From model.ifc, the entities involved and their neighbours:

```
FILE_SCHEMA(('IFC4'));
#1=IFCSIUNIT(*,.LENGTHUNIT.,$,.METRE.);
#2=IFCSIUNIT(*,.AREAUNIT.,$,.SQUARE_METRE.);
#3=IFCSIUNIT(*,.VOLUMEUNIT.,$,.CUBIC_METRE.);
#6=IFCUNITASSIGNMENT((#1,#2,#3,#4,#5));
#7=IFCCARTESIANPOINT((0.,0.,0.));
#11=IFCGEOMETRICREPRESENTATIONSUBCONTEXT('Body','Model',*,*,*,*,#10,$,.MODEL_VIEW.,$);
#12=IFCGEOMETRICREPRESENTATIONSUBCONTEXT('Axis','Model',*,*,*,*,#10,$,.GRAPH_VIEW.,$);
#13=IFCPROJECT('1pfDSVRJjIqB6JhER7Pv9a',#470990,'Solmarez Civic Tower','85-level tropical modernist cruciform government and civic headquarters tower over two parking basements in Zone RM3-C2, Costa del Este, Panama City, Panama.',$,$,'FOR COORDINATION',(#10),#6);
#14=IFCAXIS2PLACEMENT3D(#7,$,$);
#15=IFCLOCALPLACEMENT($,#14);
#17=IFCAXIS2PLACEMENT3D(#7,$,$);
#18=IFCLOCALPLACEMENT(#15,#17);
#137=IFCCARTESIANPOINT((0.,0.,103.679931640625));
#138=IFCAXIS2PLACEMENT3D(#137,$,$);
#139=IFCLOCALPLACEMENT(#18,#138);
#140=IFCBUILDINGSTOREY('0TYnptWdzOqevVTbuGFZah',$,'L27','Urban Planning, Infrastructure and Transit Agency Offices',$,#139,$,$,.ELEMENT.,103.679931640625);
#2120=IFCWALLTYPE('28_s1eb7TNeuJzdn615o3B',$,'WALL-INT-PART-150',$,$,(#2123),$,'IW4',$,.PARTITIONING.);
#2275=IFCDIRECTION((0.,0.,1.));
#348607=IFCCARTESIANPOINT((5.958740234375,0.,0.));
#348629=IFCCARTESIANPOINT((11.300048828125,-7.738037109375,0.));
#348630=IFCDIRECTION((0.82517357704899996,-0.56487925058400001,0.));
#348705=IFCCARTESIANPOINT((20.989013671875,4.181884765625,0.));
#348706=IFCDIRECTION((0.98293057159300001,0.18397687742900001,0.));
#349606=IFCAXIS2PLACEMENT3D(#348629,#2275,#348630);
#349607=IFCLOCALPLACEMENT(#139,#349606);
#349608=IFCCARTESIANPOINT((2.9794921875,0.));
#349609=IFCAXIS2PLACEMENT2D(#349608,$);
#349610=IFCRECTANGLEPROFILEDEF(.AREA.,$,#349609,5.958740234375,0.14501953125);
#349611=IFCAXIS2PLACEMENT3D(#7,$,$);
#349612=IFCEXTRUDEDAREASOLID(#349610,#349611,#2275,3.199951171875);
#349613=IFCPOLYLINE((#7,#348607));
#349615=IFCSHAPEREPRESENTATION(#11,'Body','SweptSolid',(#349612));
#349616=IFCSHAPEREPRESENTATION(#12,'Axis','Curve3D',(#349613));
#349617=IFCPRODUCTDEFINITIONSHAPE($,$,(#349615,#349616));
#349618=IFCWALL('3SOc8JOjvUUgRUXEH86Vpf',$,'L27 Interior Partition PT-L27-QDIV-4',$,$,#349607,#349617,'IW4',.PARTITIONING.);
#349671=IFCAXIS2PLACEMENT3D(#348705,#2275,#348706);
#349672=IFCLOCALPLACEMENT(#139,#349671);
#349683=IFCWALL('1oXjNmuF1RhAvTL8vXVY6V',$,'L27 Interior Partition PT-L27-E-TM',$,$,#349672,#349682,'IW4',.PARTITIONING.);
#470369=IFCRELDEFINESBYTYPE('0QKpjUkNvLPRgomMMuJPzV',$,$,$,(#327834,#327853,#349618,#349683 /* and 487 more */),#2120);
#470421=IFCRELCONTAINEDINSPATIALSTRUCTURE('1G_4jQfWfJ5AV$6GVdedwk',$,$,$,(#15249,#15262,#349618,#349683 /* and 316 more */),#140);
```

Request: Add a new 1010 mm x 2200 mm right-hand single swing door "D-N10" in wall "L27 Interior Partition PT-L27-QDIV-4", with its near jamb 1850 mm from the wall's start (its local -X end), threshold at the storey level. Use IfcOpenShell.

```python
import numpy as np
import ifcopenshell
import ifcopenshell.api.feature
import ifcopenshell.api.geometry
import ifcopenshell.api.root
import ifcopenshell.api.spatial
import ifcopenshell.geom
import ifcopenshell.util.element
import ifcopenshell.util.placement
import ifcopenshell.util.representation
import ifcopenshell.util.shape
import ifcopenshell.util.unit

model = ifcopenshell.open("model.ifc")
unit_scale = ifcopenshell.util.unit.calculate_unit_scale(model)
settings = ifcopenshell.geom.settings()


def volume(element):
    """Net volume in cubic metres, openings subtracted."""
    shape = ifcopenshell.geom.create_shape(settings, element)
    return ifcopenshell.util.shape.get_volume(shape.geometry)


wall = model.by_id(349618)
storey = ifcopenshell.util.element.get_container(wall, ifc_class="IfcBuildingStorey")
context = ifcopenshell.util.representation.get_context(model, "Model", "Body", "MODEL_VIEW")
before = volume(wall)

width, height, from_end, sill = 1.01, 2.2, 1.85, 0.0  # metres

# The wall runs along its own X axis, and the end named is its -X end.
wall_shape = ifcopenshell.geom.create_shape(settings, wall)
x, y, z = ifcopenshell.util.shape.get_vertices(wall_shape.geometry).T
start = x.min() + from_end
face, thickness = float(y.min()), float(y.max() - y.min())
wall_matrix = ifcopenshell.util.placement.get_local_placement(wall.ObjectPlacement)
level = ifcopenshell.util.placement.get_local_placement(storey.ObjectPlacement)[2, 3]


def in_wall(x, y):
    """Placement at x, y metres in the wall's axes, at sill height."""
    matrix = wall_matrix.copy()
    matrix[:, 3] = wall_matrix @ np.array([x / unit_scale, y / unit_scale, 0.0, 1.0])
    matrix[2, 3] = level + sill / unit_scale
    return matrix


# Opening: a box that overshoots both wall faces by 50 mm.
opening = ifcopenshell.api.root.create_entity(model, ifc_class="IfcOpeningElement", predefined_type="OPENING")
box = ifcopenshell.api.geometry.add_wall_representation(
    model, context=context, length=width, height=height, thickness=thickness + 0.1
)
ifcopenshell.api.geometry.assign_representation(model, product=opening, representation=box)
ifcopenshell.api.geometry.edit_object_placement(model, product=opening, matrix=in_wall(start, face - 0.05), is_si=False)
ifcopenshell.api.feature.add_feature(model, feature=opening, element=wall)

door = ifcopenshell.api.root.create_entity(model, ifc_class="IfcDoor", name="D-N10", predefined_type="DOOR")
door.OverallWidth, door.OverallHeight = width / unit_scale, height / unit_scale
door.OperationType = "SINGLE_SWING_RIGHT"
body = ifcopenshell.api.geometry.add_door_representation(
    model,
    context=context,
    overall_width=door.OverallWidth,
    overall_height=door.OverallHeight,
    operation_type="SINGLE_SWING_RIGHT",
    lining_properties={"LiningDepth": thickness / unit_scale, "ThresholdDepth": thickness / unit_scale},
)
ifcopenshell.api.geometry.assign_representation(model, product=door, representation=body)
ifcopenshell.api.spatial.assign_container(model, products=[door], relating_structure=storey)
ifcopenshell.api.feature.add_filling(model, opening=opening, element=door)

# The lining spans the wall, so the door starts at the wall face.
ifcopenshell.api.geometry.edit_object_placement(model, product=door, matrix=in_wall(start, face), is_si=False)

after = volume(wall)

print(f"wall volume {before:.3f} -> {after:.3f} m3")

model.write("model_edited.ifc")
```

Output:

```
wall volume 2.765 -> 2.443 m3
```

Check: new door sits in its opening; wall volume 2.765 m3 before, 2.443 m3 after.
